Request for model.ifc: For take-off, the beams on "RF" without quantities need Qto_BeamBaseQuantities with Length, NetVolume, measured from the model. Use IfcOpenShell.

First a look at what the model holds.

```python
import ifcopenshell
import ifcopenshell.util.element
import ifcopenshell.util.unit

model = ifcopenshell.open("model.ifc")
print(model.schema)
for unit_type in ("LENGTHUNIT", "AREAUNIT", "VOLUMEUNIT"):
    print(unit_type, ifcopenshell.util.unit.calculate_unit_scale(model, unit_type))
storey = next(s for s in model.by_type("IfcBuildingStorey") if s.Name == "RF")
beams = [e for e in ifcopenshell.util.element.get_decomposition(storey) if e.is_a("IfcBeam")]
for e in sorted(beams, key=lambda e: e.id()):
    print(e.id(), e.is_a(), e.Name, list(ifcopenshell.util.element.get_psets(e, qtos_only=True)), sep=" | ")
```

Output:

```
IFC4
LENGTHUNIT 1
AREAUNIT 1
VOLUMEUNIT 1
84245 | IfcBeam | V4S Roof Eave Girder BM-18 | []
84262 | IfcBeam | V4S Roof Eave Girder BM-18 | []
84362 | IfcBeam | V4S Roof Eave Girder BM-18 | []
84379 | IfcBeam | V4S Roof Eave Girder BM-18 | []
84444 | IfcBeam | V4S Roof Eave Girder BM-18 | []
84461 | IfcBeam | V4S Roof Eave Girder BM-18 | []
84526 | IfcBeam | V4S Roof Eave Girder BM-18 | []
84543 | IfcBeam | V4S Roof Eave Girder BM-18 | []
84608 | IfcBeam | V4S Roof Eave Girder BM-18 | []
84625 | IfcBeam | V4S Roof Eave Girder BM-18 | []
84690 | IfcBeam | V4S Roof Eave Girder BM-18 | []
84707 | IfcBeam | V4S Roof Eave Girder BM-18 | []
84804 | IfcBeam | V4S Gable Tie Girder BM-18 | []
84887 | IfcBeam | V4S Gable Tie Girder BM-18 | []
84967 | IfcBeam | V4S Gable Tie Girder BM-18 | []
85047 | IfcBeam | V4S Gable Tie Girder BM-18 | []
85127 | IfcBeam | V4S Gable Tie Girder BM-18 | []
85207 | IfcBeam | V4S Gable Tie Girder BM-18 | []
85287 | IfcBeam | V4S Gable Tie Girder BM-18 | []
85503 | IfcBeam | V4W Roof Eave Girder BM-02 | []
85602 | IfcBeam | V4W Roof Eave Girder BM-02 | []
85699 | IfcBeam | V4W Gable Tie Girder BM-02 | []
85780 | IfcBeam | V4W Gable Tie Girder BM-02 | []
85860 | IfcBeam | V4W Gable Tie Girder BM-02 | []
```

```python
import ifcopenshell
import ifcopenshell.api.pset
import ifcopenshell.geom
import ifcopenshell.util.element
import ifcopenshell.util.shape
import ifcopenshell.util.unit

model = ifcopenshell.open("model.ifc")
unit_scale = ifcopenshell.util.unit.calculate_unit_scale(model)
volume_scale = ifcopenshell.util.unit.calculate_unit_scale(model, "VOLUMEUNIT")
settings = ifcopenshell.geom.settings()

storey = next(s for s in model.by_type("IfcBuildingStorey") if s.Name == "RF")
beams = [e for e in ifcopenshell.util.element.get_decomposition(storey) if e.is_a("IfcBeam")]

for e in sorted(beams, key=lambda e: e.id()):
    if ifcopenshell.util.element.get_psets(e, qtos_only=True, should_inherit=False):
        continue
    # Geometry comes back in metres, in the element's own axes.
    shape = ifcopenshell.geom.create_shape(settings, e)
    values = {
        "Length": ifcopenshell.util.shape.get_max_xyz(shape.geometry) / unit_scale,
        "NetVolume": ifcopenshell.util.shape.get_volume(shape.geometry) / volume_scale,
    }
    qto = ifcopenshell.api.pset.add_qto(model, product=e, name="Qto_BeamBaseQuantities")
    ifcopenshell.api.pset.edit_qto(model, qto=qto, properties=values)
    print(e.id(), {k: round(v, 3) for k, v in values.items()})

model.write("model_edited.ifc")
```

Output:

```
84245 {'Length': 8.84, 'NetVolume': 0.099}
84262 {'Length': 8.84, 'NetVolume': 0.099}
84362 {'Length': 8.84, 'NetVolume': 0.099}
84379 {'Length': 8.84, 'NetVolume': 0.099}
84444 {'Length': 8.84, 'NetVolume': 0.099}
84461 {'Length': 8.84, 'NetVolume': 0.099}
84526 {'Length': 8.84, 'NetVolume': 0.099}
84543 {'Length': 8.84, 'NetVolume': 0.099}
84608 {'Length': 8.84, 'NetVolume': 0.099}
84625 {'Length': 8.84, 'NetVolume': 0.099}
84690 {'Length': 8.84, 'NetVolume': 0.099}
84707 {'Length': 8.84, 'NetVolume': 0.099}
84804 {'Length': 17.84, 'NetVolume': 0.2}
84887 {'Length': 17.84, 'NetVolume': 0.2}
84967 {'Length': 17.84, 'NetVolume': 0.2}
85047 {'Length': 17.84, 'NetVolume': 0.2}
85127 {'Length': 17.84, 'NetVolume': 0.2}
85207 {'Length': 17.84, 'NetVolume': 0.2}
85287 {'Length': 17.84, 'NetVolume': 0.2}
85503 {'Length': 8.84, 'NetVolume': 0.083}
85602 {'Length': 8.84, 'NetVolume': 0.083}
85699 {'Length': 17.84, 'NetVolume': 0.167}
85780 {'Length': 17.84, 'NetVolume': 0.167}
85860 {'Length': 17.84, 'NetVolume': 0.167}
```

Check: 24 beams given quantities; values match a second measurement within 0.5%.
